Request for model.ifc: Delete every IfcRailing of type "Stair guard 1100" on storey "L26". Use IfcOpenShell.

First a look at what the model holds.

```python
import ifcopenshell
import ifcopenshell.util.element

model = ifcopenshell.open("model.ifc")
print(model.schema)
storey = next(s for s in model.by_type("IfcBuildingStorey") if s.Name == "L26")
railings = [e for e in ifcopenshell.util.element.get_decomposition(storey) if e.is_a("IfcRailing")]
seen = {}
for e in railings:
    element_type = ifcopenshell.util.element.get_type(e)
    name = element_type.Name if element_type not in (None, e) else None
    seen[name] = seen.get(name, 0) + 1
for name, count in sorted(seen.items(), key=str):
    print(count, "x", name)
```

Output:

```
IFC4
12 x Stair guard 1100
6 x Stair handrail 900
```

```python
import ifcopenshell
import ifcopenshell.api.root
import ifcopenshell.util.element

model = ifcopenshell.open("model.ifc")

storey = next(s for s in model.by_type("IfcBuildingStorey") if s.Name == "L26")
railings = [e for e in ifcopenshell.util.element.get_decomposition(storey) if e.is_a("IfcRailing")]
targets = [e for e in railings if (t := ifcopenshell.util.element.get_type(e)) not in (None, e) and t.Name == "Stair guard 1100"]

for e in targets:
    ifcopenshell.api.root.remove_product(model, product=e)
print(len(targets), "removed")

model.write("model-out.ifc")
```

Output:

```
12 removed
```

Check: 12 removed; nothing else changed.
